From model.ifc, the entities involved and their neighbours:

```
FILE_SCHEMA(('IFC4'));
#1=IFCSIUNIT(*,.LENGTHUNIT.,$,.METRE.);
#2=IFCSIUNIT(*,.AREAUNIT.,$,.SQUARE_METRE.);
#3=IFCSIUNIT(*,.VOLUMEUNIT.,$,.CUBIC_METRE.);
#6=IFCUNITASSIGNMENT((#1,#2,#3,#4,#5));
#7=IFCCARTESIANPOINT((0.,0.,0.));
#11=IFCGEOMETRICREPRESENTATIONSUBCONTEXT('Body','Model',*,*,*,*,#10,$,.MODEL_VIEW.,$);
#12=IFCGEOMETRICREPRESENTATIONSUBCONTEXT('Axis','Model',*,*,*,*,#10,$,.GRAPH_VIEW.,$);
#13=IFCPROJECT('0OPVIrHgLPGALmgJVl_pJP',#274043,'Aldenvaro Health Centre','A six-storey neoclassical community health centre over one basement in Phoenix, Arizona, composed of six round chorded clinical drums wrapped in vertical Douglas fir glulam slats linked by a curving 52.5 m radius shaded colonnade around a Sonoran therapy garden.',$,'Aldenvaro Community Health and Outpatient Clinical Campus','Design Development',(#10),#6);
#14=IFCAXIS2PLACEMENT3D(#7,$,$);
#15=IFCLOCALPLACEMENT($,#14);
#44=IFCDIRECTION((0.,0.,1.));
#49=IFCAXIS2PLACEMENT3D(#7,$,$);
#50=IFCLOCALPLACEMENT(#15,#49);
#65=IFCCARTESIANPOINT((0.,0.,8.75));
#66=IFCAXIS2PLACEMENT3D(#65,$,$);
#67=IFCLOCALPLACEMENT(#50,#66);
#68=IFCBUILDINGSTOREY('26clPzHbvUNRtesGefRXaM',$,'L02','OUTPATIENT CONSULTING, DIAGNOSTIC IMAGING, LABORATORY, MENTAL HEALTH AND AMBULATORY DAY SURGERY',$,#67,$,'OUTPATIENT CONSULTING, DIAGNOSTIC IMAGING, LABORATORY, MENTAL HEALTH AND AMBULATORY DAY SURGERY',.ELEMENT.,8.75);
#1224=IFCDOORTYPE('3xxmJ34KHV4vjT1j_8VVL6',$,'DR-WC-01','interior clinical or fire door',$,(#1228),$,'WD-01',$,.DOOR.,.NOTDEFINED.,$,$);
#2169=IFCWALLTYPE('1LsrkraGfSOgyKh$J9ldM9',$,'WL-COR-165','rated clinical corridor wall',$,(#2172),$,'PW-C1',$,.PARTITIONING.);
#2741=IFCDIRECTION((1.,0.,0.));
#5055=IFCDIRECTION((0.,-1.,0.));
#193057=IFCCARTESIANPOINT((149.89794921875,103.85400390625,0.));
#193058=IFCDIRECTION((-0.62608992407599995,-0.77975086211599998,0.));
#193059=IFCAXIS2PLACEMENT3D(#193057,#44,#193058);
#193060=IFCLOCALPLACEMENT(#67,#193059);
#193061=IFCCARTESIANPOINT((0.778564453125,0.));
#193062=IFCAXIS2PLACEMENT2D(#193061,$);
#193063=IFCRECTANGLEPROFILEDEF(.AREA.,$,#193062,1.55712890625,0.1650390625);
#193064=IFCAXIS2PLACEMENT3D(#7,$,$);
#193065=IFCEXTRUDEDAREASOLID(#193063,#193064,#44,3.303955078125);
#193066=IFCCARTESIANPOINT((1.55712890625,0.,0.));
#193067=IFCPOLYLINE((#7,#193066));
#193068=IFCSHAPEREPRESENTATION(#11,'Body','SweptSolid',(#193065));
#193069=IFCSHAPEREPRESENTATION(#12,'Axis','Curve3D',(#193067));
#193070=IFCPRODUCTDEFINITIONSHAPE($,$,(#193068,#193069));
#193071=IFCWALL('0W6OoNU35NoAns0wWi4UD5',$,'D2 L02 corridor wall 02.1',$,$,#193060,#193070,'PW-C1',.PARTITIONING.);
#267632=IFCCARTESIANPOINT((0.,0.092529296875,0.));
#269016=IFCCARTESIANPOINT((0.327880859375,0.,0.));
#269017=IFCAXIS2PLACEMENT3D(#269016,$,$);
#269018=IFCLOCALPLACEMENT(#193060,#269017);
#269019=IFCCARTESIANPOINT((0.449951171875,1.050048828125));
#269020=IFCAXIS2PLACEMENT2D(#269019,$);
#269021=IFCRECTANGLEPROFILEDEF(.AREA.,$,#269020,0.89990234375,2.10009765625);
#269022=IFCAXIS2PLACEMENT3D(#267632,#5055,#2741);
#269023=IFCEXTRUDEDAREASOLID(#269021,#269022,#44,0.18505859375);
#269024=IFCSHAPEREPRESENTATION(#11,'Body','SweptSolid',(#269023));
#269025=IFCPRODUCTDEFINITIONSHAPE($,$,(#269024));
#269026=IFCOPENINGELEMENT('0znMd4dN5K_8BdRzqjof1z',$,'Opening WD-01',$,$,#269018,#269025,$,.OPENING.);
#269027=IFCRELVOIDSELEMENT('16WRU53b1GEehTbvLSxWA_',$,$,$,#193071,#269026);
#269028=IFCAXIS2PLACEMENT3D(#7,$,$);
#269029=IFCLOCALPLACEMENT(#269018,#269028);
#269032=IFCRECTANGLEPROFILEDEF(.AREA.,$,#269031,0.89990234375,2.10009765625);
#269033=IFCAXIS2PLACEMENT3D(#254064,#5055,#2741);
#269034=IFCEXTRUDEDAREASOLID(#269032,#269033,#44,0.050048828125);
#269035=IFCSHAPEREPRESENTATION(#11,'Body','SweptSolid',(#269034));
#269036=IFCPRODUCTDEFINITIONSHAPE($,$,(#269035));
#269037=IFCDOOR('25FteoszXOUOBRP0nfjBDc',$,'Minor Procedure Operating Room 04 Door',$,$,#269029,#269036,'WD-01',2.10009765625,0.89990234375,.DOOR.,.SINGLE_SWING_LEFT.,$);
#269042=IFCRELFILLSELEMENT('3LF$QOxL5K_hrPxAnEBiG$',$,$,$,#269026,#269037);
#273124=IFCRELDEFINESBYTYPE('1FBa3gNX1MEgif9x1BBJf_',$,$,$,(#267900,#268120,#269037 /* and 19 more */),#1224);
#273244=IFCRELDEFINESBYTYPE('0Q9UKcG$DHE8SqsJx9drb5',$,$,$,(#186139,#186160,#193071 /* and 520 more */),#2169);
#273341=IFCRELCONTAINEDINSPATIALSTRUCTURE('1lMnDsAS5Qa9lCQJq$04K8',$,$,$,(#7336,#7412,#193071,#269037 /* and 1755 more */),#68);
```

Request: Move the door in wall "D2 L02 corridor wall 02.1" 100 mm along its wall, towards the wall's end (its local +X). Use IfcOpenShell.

```python
import ifcopenshell
import ifcopenshell.api.geometry
import ifcopenshell.util.placement
import ifcopenshell.util.unit

model = ifcopenshell.open("model.ifc")
unit_scale = ifcopenshell.util.unit.calculate_unit_scale(model)

door = model.by_guid("25FteoszXOUOBRP0nfjBDc")
opening = door.FillsVoids[0].RelatingOpeningElement
wall = opening.VoidsElements[0].RelatingBuildingElement

wall_matrix = ifcopenshell.util.placement.get_local_placement(wall.ObjectPlacement)
shift = wall_matrix[:3, 0] * 0.1 / unit_scale
before = ifcopenshell.util.placement.get_local_placement(door.ObjectPlacement)[:3, 3].copy()

# The door is placed relative to its opening, so it follows when the opening moves.
matrix = ifcopenshell.util.placement.get_local_placement(opening.ObjectPlacement)
matrix[:3, 3] += shift
ifcopenshell.api.geometry.edit_object_placement(
    model, product=opening, matrix=matrix, is_si=False, should_transform_children=True
)

after = ifcopenshell.util.placement.get_local_placement(door.ObjectPlacement)[:3, 3]
print("door moved by", (after - before).round(3) + 0.0)

model.write("model_v2.ifc")
```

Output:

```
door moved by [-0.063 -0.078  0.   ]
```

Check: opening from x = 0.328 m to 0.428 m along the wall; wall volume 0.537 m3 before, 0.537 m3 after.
